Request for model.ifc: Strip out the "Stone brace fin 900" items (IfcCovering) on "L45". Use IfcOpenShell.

First a look at what the model holds.

```python
import ifcopenshell
import ifcopenshell.util.element

model = ifcopenshell.open("model.ifc")
print(model.schema)
storey = next(s for s in model.by_type("IfcBuildingStorey") if s.Name == "L45")
coverings = [e for e in ifcopenshell.util.element.get_decomposition(storey) if e.is_a("IfcCovering")]
seen = {}
for e in coverings:
    element_type = ifcopenshell.util.element.get_type(e)
    name = element_type.Name if element_type not in (None, e) else None
    seen[name] = seen.get(name, 0) + 1
for name, count in sorted(seen.items(), key=str):
    print(count, "x", name)
```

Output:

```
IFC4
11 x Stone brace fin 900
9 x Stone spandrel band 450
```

```python
import ifcopenshell
import ifcopenshell.api.root
import ifcopenshell.util.element

model = ifcopenshell.open("model.ifc")

storey = next(s for s in model.by_type("IfcBuildingStorey") if s.Name == "L45")
coverings = [e for e in ifcopenshell.util.element.get_decomposition(storey) if e.is_a("IfcCovering")]
targets = [e for e in coverings if (t := ifcopenshell.util.element.get_type(e)) not in (None, e) and t.Name == "Stone brace fin 900"]

for e in targets:
    ifcopenshell.api.root.remove_product(model, product=e)
print(len(targets), "removed")

model.write("model_rev.ifc")
```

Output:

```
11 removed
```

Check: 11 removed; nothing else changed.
